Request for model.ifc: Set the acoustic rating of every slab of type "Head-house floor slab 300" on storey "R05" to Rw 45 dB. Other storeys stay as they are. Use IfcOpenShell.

First a look at what the model holds.

```python
import ifcopenshell
import ifcopenshell.util.element

model = ifcopenshell.open("model.ifc")
print(model.schema)
storey = next(s for s in model.by_type("IfcBuildingStorey") if s.Name == "R05")
slabs = [e for e in ifcopenshell.util.element.get_decomposition(storey) if e.is_a("IfcSlab")]
seen = {}
for e in slabs:
    element_type = ifcopenshell.util.element.get_type(e)
    key = (element_type.Name if element_type != e and element_type else None, ifcopenshell.util.element.get_pset(e, "Pset_SlabCommon", "AcousticRating"))
    seen[key] = seen.get(key, 0) + 1
for (name, value), count in sorted(seen.items(), key=str):
    print(count, "x", name, "|", value)
```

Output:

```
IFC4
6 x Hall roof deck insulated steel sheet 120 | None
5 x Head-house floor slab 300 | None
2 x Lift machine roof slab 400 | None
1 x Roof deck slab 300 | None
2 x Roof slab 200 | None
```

```python
import ifcopenshell
import ifcopenshell.api.pset
import ifcopenshell.util.element

model = ifcopenshell.open("model.ifc")

storey = next(s for s in model.by_type("IfcBuildingStorey") if s.Name == "R05")
slabs = [e for e in ifcopenshell.util.element.get_decomposition(storey) if e.is_a("IfcSlab")]

count = 0
for e in slabs:
    element_type = ifcopenshell.util.element.get_type(e)
    if element_type in (None, e) or element_type.Name != "Head-house floor slab 300":
        continue
    # add_pset returns the element's existing set when there is one.
    pset = ifcopenshell.api.pset.add_pset(model, product=e, name="Pset_SlabCommon")
    ifcopenshell.api.pset.edit_pset(model, pset=pset, properties={"AcousticRating": "Rw 45 dB"})
    count += 1

print(count, "slabs updated")

model.write("model_edited.ifc")
```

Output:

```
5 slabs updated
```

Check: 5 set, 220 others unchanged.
